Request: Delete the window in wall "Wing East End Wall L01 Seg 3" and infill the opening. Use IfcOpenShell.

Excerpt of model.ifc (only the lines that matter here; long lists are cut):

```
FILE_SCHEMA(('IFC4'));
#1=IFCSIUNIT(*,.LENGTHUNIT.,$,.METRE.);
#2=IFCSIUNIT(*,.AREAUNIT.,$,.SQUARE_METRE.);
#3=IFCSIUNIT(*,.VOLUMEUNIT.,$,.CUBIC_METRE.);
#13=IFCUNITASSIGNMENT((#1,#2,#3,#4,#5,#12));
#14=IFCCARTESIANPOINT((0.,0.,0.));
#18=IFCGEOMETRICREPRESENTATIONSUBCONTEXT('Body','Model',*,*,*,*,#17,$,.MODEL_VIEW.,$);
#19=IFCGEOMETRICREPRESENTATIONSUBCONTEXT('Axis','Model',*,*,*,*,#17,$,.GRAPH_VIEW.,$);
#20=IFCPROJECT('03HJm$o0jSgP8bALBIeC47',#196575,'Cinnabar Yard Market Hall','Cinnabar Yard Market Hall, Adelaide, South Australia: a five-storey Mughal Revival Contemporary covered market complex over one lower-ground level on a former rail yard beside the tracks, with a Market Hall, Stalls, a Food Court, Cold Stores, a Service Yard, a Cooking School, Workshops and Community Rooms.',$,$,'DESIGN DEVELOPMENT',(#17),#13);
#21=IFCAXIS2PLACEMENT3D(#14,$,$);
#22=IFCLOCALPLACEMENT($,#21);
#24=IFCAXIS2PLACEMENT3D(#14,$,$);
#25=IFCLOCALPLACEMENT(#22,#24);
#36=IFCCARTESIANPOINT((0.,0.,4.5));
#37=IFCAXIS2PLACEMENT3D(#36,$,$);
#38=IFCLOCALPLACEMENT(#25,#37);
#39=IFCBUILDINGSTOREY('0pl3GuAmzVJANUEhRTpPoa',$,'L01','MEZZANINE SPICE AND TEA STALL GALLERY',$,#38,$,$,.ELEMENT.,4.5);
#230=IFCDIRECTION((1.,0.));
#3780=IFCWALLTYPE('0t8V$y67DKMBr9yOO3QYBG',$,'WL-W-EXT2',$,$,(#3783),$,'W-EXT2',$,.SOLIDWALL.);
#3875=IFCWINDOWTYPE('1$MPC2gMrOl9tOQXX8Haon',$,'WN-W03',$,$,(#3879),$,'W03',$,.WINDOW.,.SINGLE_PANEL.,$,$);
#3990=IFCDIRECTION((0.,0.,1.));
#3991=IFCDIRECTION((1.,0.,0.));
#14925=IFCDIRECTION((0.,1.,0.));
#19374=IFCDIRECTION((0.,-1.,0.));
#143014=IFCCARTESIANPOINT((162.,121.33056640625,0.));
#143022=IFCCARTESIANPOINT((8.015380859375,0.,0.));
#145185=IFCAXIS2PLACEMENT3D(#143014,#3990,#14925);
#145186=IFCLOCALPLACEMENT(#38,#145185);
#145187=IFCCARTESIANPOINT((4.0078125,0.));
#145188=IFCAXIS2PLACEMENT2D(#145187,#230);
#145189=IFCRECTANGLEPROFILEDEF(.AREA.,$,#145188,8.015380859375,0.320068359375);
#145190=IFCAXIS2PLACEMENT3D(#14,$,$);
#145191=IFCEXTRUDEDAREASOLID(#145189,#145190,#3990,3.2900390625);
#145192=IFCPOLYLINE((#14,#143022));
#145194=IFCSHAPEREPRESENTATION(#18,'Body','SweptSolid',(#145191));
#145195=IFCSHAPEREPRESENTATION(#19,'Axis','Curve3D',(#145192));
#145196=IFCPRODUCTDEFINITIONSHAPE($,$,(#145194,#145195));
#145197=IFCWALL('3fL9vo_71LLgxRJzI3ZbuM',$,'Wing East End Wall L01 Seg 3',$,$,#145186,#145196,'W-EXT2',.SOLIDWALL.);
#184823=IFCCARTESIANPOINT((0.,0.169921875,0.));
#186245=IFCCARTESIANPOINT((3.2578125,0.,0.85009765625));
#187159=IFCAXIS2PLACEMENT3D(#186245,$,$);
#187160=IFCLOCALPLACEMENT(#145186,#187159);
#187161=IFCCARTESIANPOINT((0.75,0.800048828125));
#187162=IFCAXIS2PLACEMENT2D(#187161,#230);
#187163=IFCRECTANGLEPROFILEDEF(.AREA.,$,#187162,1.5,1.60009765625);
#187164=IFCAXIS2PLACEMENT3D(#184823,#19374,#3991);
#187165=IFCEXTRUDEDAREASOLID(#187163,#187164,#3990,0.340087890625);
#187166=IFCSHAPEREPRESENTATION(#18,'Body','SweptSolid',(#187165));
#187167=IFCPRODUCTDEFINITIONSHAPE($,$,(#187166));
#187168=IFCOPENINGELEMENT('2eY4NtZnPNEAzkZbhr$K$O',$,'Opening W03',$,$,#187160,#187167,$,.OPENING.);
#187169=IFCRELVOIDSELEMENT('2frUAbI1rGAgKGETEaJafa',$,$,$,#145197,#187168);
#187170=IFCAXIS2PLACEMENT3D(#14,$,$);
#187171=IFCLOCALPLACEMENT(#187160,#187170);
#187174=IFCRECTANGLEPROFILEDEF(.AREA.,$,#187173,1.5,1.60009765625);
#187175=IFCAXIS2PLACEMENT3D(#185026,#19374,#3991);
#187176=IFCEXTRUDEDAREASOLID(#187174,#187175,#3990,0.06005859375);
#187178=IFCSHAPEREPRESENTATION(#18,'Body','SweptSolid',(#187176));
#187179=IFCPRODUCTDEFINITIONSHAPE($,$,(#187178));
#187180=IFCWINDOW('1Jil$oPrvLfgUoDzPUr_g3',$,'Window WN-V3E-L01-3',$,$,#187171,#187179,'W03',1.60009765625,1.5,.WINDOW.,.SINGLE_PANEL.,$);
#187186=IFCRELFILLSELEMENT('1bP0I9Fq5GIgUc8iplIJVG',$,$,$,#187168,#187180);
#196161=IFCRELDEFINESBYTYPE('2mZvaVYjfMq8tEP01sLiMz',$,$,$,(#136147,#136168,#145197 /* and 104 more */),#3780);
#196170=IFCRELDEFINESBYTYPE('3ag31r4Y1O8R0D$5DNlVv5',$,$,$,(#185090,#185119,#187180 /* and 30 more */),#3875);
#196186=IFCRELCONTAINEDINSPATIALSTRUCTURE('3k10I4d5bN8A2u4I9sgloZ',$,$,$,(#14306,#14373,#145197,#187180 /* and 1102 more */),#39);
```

```python
import ifcopenshell
import ifcopenshell.api.feature
import ifcopenshell.api.root
import ifcopenshell.geom
import ifcopenshell.util.shape

model = ifcopenshell.open("model.ifc")
settings = ifcopenshell.geom.settings()


def volume(element):
    """Net volume in cubic metres, openings subtracted."""
    shape = ifcopenshell.geom.create_shape(settings, element)
    return ifcopenshell.util.shape.get_volume(shape.geometry)


window = model.by_guid("1Jil$oPrvLfgUoDzPUr_g3")
opening = window.FillsVoids[0].RelatingOpeningElement
wall = opening.VoidsElements[0].RelatingBuildingElement
before = volume(wall)

ifcopenshell.api.root.remove_product(model, product=window)
ifcopenshell.api.feature.remove_feature(model, feature=opening)

after = volume(wall)

print(f"wall volume {before:.3f} -> {after:.3f} m3")

model.write("model_updated.ifc")
```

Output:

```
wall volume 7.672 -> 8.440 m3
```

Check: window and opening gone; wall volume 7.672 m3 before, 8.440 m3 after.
